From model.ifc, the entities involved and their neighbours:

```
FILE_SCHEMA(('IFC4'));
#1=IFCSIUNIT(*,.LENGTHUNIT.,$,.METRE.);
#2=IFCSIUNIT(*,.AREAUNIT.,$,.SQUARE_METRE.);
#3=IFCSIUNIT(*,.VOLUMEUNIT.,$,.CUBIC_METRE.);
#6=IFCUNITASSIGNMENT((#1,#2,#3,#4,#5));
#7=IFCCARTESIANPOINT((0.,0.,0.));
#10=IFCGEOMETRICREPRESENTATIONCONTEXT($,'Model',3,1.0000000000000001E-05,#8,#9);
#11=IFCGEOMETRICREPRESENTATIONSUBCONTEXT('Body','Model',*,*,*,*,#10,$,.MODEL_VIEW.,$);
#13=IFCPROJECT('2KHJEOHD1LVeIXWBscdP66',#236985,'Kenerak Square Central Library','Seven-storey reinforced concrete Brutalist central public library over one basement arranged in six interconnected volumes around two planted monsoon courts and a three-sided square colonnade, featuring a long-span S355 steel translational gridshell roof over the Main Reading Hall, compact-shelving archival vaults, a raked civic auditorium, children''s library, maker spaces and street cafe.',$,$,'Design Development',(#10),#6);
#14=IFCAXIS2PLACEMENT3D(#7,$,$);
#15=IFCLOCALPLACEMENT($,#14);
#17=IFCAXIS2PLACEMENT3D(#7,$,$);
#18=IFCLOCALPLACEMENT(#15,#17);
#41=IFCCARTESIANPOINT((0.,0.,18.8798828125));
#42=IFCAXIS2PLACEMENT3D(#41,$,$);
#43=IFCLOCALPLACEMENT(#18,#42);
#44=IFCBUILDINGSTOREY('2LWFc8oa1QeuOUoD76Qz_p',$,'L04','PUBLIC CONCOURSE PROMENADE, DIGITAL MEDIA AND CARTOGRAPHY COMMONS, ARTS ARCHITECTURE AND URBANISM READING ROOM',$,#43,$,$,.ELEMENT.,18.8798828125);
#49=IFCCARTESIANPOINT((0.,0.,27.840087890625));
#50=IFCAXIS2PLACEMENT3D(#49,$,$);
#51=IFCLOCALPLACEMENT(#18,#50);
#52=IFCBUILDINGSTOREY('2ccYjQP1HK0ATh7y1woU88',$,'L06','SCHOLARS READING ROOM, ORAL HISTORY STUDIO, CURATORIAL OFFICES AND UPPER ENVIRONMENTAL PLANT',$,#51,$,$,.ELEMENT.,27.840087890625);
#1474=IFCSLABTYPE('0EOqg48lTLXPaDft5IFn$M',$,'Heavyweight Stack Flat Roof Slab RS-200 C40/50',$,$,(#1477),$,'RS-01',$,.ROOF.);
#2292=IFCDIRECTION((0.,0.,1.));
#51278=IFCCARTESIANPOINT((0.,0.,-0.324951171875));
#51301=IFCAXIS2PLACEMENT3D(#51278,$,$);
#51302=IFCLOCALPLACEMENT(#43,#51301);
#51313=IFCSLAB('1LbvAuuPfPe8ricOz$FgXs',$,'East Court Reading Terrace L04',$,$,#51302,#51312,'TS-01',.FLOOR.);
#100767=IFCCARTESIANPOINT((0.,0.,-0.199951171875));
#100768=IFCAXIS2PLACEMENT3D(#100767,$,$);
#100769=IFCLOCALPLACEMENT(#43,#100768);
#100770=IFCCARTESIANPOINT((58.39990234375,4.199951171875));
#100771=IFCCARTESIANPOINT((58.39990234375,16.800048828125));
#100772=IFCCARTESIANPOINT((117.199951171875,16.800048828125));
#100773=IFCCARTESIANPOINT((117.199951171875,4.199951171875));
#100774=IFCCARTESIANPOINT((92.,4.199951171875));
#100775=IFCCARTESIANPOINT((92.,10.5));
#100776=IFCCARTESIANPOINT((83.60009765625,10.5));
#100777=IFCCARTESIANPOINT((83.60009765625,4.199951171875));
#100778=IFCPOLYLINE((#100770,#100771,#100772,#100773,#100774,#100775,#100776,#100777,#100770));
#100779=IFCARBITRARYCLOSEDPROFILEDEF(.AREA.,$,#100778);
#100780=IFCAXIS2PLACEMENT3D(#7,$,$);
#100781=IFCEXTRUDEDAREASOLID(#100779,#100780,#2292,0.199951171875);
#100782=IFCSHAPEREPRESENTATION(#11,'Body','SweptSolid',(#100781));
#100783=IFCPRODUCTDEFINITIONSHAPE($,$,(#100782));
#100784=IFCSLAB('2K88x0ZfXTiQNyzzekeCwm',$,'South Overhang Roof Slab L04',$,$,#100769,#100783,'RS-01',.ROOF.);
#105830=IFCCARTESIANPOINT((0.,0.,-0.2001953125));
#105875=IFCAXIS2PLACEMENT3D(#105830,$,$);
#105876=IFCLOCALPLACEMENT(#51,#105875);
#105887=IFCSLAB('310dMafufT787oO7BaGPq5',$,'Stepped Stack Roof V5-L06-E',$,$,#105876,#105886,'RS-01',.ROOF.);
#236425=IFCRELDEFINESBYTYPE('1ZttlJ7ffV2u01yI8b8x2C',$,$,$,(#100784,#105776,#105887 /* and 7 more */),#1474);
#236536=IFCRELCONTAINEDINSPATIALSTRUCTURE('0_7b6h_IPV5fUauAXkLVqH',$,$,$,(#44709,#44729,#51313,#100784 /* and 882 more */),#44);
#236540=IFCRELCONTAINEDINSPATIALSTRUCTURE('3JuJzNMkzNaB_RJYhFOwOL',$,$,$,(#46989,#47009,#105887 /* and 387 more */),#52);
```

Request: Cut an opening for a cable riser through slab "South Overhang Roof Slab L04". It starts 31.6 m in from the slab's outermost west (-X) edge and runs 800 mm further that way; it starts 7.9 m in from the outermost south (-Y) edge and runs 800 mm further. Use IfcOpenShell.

```python
import numpy as np
import ifcopenshell
import ifcopenshell.api.feature
import ifcopenshell.api.geometry
import ifcopenshell.api.root
import ifcopenshell.geom
import ifcopenshell.util.placement
import ifcopenshell.util.representation
import ifcopenshell.util.shape
import ifcopenshell.util.unit

model = ifcopenshell.open("model.ifc")
unit_scale = ifcopenshell.util.unit.calculate_unit_scale(model)
settings = ifcopenshell.geom.settings()


def volume(element):
    """Net volume in cubic metres, openings subtracted."""
    shape = ifcopenshell.geom.create_shape(settings, element)
    return ifcopenshell.util.shape.get_volume(shape.geometry)


slab = model.by_guid("2K88x0ZfXTiQNyzzekeCwm")
before = volume(slab)

# Extent in the slab's own axes, in metres. The edges named are its -X and -Y sides.
slab_shape = ifcopenshell.geom.create_shape(settings, slab)
vertices = ifcopenshell.util.shape.get_vertices(slab_shape.geometry)
x_min, y_min, bottom = vertices.min(axis=0)
top = vertices[:, 2].max()

opening = ifcopenshell.api.root.create_entity(model, ifc_class="IfcOpeningElement", name="Cable riser opening", predefined_type="OPENING")
context = ifcopenshell.util.representation.get_context(model, "Model", "Body", "MODEL_VIEW")
width, depth = 0.8, 0.8
outline = [(0.0, 0.0), (width, 0.0), (width, depth), (0.0, depth), (0.0, 0.0)]
# Overshoot both faces by 50 mm so the cut is clean.
shape = ifcopenshell.api.geometry.add_slab_representation(
    model, context=context, depth=top - bottom + 0.1, polyline=outline
)
ifcopenshell.api.geometry.assign_representation(model, product=opening, representation=shape)

matrix = ifcopenshell.util.placement.get_local_placement(slab.ObjectPlacement)
matrix[:, 3] = matrix @ np.append(np.array([x_min + 31.6, y_min + 7.9, bottom - 0.05]) / unit_scale, 1.0)
ifcopenshell.api.geometry.edit_object_placement(model, product=opening, matrix=matrix, is_si=False)
ifcopenshell.api.feature.add_feature(model, feature=opening, element=slab)

after = volume(slab)

print(f"slab volume {before:.3f} -> {after:.3f} m3")

model.write("model-out.ifc")
```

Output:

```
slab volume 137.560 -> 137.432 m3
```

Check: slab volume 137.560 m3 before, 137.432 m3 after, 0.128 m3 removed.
